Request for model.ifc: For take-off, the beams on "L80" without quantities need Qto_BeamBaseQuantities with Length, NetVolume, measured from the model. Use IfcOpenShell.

First a look at what the model holds.

```python
import ifcopenshell
import ifcopenshell.util.element
import ifcopenshell.util.unit

model = ifcopenshell.open("model.ifc")
print(model.schema)
for unit_type in ("LENGTHUNIT", "AREAUNIT", "VOLUMEUNIT"):
    print(unit_type, ifcopenshell.util.unit.calculate_unit_scale(model, unit_type))
storey = next(s for s in model.by_type("IfcBuildingStorey") if s.Name == "L80")
beams = [e for e in ifcopenshell.util.element.get_decomposition(storey) if e.is_a("IfcBeam")]
for e in sorted(beams, key=lambda e: e.id()):
    print(e.id(), e.is_a(), e.Name, list(ifcopenshell.util.element.get_psets(e, qtos_only=True)), sep=" | ")
```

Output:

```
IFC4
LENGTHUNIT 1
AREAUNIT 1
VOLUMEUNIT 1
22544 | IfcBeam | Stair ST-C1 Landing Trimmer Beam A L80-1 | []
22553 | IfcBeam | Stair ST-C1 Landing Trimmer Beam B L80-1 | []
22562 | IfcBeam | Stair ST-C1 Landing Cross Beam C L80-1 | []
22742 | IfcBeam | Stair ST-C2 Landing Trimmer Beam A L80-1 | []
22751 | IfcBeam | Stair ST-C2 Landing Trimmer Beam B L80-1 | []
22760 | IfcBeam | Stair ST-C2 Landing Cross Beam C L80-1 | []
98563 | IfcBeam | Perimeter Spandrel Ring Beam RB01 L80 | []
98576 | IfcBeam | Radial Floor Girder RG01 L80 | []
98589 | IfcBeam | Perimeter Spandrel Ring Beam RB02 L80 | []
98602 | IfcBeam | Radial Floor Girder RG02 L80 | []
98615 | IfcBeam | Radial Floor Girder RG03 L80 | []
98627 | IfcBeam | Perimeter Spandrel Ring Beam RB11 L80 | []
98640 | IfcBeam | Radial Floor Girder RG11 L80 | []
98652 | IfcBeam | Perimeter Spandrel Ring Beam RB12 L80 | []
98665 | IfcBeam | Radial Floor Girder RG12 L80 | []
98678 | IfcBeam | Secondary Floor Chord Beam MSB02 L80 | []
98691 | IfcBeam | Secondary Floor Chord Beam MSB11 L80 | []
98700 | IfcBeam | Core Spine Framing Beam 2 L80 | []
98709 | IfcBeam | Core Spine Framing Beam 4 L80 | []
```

```python
import ifcopenshell
import ifcopenshell.api.pset
import ifcopenshell.geom
import ifcopenshell.util.element
import ifcopenshell.util.shape
import ifcopenshell.util.unit

model = ifcopenshell.open("model.ifc")
unit_scale = ifcopenshell.util.unit.calculate_unit_scale(model)
volume_scale = ifcopenshell.util.unit.calculate_unit_scale(model, "VOLUMEUNIT")
settings = ifcopenshell.geom.settings()

storey = next(s for s in model.by_type("IfcBuildingStorey") if s.Name == "L80")
beams = [e for e in ifcopenshell.util.element.get_decomposition(storey) if e.is_a("IfcBeam")]

for e in sorted(beams, key=lambda e: e.id()):
    if ifcopenshell.util.element.get_psets(e, qtos_only=True, should_inherit=False):
        continue
    # Geometry comes back in metres, in the element's own axes.
    shape = ifcopenshell.geom.create_shape(settings, e)
    values = {
        "Length": ifcopenshell.util.shape.get_max_xyz(shape.geometry) / unit_scale,
        "NetVolume": ifcopenshell.util.shape.get_volume(shape.geometry) / volume_scale,
    }
    qto = ifcopenshell.api.pset.add_qto(model, product=e, name="Qto_BeamBaseQuantities")
    ifcopenshell.api.pset.edit_qto(model, qto=qto, properties=values)
    print(e.id(), {k: round(v, 3) for k, v in values.items()})

model.write("model_edited.ifc")
```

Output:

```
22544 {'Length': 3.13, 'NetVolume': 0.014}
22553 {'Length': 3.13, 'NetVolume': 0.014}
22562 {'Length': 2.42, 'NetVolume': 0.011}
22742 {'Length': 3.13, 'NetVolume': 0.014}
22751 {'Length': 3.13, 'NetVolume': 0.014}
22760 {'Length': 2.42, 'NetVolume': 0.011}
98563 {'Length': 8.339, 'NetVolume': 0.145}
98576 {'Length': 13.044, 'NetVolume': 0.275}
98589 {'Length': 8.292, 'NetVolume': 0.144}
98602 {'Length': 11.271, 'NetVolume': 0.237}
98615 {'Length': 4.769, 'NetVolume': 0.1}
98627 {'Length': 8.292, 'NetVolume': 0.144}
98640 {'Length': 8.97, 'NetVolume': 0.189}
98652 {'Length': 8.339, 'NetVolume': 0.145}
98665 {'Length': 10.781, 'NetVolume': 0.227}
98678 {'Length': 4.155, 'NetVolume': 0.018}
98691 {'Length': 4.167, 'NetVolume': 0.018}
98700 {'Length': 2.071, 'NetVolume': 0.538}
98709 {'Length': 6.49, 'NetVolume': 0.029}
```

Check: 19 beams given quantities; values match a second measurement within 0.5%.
